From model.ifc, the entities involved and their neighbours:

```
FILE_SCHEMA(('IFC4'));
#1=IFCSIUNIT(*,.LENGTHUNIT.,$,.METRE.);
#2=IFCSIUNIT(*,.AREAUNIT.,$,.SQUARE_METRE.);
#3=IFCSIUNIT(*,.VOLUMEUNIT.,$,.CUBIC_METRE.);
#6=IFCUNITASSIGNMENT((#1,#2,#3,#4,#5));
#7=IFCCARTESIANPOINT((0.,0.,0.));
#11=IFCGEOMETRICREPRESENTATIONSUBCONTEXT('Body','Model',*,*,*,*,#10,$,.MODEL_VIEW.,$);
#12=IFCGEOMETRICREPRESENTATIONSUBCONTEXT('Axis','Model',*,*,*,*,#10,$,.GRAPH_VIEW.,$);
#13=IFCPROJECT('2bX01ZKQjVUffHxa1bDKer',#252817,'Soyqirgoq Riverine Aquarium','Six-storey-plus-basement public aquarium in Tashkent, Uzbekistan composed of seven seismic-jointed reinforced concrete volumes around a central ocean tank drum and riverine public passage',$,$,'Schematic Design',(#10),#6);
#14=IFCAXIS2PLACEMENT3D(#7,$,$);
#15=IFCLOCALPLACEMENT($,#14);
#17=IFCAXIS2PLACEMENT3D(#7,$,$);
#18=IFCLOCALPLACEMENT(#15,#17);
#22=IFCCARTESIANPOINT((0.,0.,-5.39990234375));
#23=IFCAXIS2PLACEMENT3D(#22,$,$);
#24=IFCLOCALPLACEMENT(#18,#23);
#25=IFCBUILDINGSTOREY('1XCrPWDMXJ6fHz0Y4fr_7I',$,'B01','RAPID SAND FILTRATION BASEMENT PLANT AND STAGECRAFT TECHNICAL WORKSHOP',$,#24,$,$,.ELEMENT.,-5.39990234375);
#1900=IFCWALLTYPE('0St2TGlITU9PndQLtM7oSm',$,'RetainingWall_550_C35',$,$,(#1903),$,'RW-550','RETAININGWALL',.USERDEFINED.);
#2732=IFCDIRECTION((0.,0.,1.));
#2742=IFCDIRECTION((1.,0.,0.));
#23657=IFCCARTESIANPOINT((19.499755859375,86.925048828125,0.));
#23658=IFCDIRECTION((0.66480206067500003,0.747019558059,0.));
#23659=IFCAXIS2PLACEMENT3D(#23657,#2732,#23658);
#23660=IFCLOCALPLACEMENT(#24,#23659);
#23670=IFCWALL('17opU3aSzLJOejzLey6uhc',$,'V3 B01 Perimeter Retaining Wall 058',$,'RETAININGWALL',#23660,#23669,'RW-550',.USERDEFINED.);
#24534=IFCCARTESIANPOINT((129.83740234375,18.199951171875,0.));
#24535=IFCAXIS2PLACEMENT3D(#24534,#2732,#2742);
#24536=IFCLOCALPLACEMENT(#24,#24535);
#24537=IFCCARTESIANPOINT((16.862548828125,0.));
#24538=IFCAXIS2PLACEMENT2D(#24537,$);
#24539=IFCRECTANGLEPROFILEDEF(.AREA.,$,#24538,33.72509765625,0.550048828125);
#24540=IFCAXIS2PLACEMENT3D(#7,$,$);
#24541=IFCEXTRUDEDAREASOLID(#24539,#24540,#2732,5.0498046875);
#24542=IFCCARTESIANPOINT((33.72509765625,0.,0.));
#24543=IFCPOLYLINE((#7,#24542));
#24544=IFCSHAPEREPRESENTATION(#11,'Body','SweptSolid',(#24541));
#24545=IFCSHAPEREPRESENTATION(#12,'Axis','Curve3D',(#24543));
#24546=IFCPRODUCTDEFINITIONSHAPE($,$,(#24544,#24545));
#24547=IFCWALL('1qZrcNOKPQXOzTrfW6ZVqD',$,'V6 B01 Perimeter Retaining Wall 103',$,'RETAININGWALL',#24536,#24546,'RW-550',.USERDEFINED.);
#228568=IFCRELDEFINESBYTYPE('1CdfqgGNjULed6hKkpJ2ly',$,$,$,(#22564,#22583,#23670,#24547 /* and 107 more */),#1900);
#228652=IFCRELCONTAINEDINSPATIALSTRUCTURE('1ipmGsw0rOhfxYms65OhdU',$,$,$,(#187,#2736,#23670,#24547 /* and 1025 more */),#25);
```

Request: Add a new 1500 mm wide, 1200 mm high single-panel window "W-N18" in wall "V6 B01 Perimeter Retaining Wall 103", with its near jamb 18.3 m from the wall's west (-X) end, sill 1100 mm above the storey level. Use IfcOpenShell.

```python
import numpy as np
import ifcopenshell
import ifcopenshell.api.feature
import ifcopenshell.api.geometry
import ifcopenshell.api.root
import ifcopenshell.api.spatial
import ifcopenshell.geom
import ifcopenshell.util.element
import ifcopenshell.util.placement
import ifcopenshell.util.representation
import ifcopenshell.util.shape
import ifcopenshell.util.unit

model = ifcopenshell.open("model.ifc")
unit_scale = ifcopenshell.util.unit.calculate_unit_scale(model)
settings = ifcopenshell.geom.settings()


def volume(element):
    """Net volume in cubic metres, openings subtracted."""
    shape = ifcopenshell.geom.create_shape(settings, element)
    return ifcopenshell.util.shape.get_volume(shape.geometry)


wall = model.by_guid("1qZrcNOKPQXOzTrfW6ZVqD")
storey = ifcopenshell.util.element.get_container(wall, ifc_class="IfcBuildingStorey")
context = ifcopenshell.util.representation.get_context(model, "Model", "Body", "MODEL_VIEW")
before = volume(wall)

width, height, from_end, sill = 1.5, 1.2, 18.3, 1.1  # metres

# The wall runs along its own X axis, and the end named is its -X end.
wall_shape = ifcopenshell.geom.create_shape(settings, wall)
x, y, z = ifcopenshell.util.shape.get_vertices(wall_shape.geometry).T
start = x.min() + from_end
face, thickness = float(y.min()), float(y.max() - y.min())
wall_matrix = ifcopenshell.util.placement.get_local_placement(wall.ObjectPlacement)
level = ifcopenshell.util.placement.get_local_placement(storey.ObjectPlacement)[2, 3]


def in_wall(x, y):
    """Placement at x, y metres in the wall's axes, at sill height."""
    matrix = wall_matrix.copy()
    matrix[:, 3] = wall_matrix @ np.array([x / unit_scale, y / unit_scale, 0.0, 1.0])
    matrix[2, 3] = level + sill / unit_scale
    return matrix


# Opening: a box that overshoots both wall faces by 50 mm.
opening = ifcopenshell.api.root.create_entity(model, ifc_class="IfcOpeningElement", predefined_type="OPENING")
box = ifcopenshell.api.geometry.add_wall_representation(
    model, context=context, length=width, height=height, thickness=thickness + 0.1
)
ifcopenshell.api.geometry.assign_representation(model, product=opening, representation=box)
ifcopenshell.api.geometry.edit_object_placement(model, product=opening, matrix=in_wall(start, face - 0.05), is_si=False)
ifcopenshell.api.feature.add_feature(model, feature=opening, element=wall)

window = ifcopenshell.api.root.create_entity(model, ifc_class="IfcWindow", name="W-N18", predefined_type="WINDOW")
window.OverallWidth, window.OverallHeight = width / unit_scale, height / unit_scale
window.PartitioningType = "SINGLE_PANEL"
body = ifcopenshell.api.geometry.add_window_representation(
    model,
    context=context,
    overall_width=window.OverallWidth,
    overall_height=window.OverallHeight,
    partition_type="SINGLE_PANEL",
)
ifcopenshell.api.geometry.assign_representation(model, product=window, representation=body)
ifcopenshell.api.spatial.assign_container(model, products=[window], relating_structure=storey)
ifcopenshell.api.feature.add_filling(model, opening=opening, element=window)

# Centre the window in the wall's thickness.
ifcopenshell.api.geometry.edit_object_placement(model, product=window, matrix=in_wall(start, face), is_si=False)
window_shape = ifcopenshell.geom.create_shape(settings, window)
depth = ifcopenshell.util.shape.get_vertices(window_shape.geometry)[:, 1]
offset = face + thickness / 2 - (depth.min() + depth.max()) / 2
ifcopenshell.api.geometry.edit_object_placement(model, product=window, matrix=in_wall(start, offset), is_si=False)

after = volume(wall)

print(f"wall volume {before:.3f} -> {after:.3f} m3")

model.write("model_edited.ifc")
```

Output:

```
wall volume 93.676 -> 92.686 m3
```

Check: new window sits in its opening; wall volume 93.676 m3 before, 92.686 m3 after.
